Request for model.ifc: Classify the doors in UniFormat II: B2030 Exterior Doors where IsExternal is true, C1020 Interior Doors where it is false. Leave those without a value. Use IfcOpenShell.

First a look at what the model holds.

```python
import ifcopenshell
import ifcopenshell.util.element

model = ifcopenshell.open("model.ifc")
print(model.schema)
print("classifications:", [c.Name for c in model.by_type("IfcClassification")])
values = [ifcopenshell.util.element.get_pset(e, "Pset_DoorCommon", "IsExternal") for e in model.by_type("IfcDoor")]
for value in (True, False, None):
    print("IsExternal", value, values.count(value))
```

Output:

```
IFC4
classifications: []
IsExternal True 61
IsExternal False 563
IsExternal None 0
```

```python
import ifcopenshell
import ifcopenshell.api.classification
import ifcopenshell.util.element

model = ifcopenshell.open("model.ifc")

system = ifcopenshell.api.classification.add_classification(model, classification="UniFormat II")

doors = model.by_type("IfcDoor")
external = {e: ifcopenshell.util.element.get_pset(e, "Pset_DoorCommon", "IsExternal") for e in doors}
for flag, code, name in ((True, "B2030", "Exterior Doors"), (False, "C1020", "Interior Doors")):
    products = [e for e in doors if external[e] is flag]
    ifcopenshell.api.classification.add_reference(
        model, products=products, classification=system, identification=code, name=name
    )
    print(code, len(products))

model.write("model_v2.ifc")
```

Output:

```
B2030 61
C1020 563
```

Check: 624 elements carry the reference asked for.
